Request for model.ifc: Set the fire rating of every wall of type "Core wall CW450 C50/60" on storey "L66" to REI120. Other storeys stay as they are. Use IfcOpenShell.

First a look at what the model holds.

```python
import ifcopenshell
import ifcopenshell.util.element

model = ifcopenshell.open("model.ifc")
print(model.schema)
storey = next(s for s in model.by_type("IfcBuildingStorey") if s.Name == "L66")
walls = [e for e in ifcopenshell.util.element.get_decomposition(storey) if e.is_a("IfcWall")]
seen = {}
for e in walls:
    element_type = ifcopenshell.util.element.get_type(e)
    key = (element_type.Name if element_type != e and element_type else None, ifcopenshell.util.element.get_pset(e, "Pset_WallCommon", "FireRating"))
    seen[key] = seen.get(key, 0) + 1
for (name, value), count in sorted(seen.items(), key=str):
    print(count, "x", name, "|", value)
```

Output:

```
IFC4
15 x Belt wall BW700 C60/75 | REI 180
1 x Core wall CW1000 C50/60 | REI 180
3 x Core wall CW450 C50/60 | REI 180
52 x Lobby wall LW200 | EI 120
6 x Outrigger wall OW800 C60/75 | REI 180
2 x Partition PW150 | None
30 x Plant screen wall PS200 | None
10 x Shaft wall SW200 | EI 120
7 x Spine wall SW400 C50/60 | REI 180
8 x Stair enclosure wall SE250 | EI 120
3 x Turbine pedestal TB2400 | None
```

```python
import ifcopenshell
import ifcopenshell.api.pset
import ifcopenshell.util.element

model = ifcopenshell.open("model.ifc")

storey = next(s for s in model.by_type("IfcBuildingStorey") if s.Name == "L66")
walls = [e for e in ifcopenshell.util.element.get_decomposition(storey) if e.is_a("IfcWall")]

count = 0
for e in walls:
    element_type = ifcopenshell.util.element.get_type(e)
    if element_type in (None, e) or element_type.Name != "Core wall CW450 C50/60":
        continue
    # add_pset returns the element's existing set when there is one.
    pset = ifcopenshell.api.pset.add_pset(model, product=e, name="Pset_WallCommon")
    ifcopenshell.api.pset.edit_pset(model, pset=pset, properties={"FireRating": "REI120"})
    count += 1

print(count, "walls updated")

model.write("model_v2.ifc")
```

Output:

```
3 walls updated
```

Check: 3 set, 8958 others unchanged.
